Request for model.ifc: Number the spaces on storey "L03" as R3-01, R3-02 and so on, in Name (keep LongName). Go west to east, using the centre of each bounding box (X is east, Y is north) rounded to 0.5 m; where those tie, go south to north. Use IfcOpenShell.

First a look at what the model holds.

```python
import ifcopenshell
import ifcopenshell.util.element
import ifcopenshell.util.placement

model = ifcopenshell.open("model.ifc")
print(model.schema)
storey = next(s for s in model.by_type("IfcBuildingStorey") if s.Name == "L03")
spaces = [e for e in ifcopenshell.util.element.get_decomposition(storey) if e.is_a("IfcSpace")]
for e in sorted(spaces, key=lambda e: e.id()):
    origin = ifcopenshell.util.placement.get_local_placement(e.ObjectPlacement)[:3, 3]
    print(e.id(), e.Name, e.LongName, origin.round(2) + 0.0, sep=" | ")
```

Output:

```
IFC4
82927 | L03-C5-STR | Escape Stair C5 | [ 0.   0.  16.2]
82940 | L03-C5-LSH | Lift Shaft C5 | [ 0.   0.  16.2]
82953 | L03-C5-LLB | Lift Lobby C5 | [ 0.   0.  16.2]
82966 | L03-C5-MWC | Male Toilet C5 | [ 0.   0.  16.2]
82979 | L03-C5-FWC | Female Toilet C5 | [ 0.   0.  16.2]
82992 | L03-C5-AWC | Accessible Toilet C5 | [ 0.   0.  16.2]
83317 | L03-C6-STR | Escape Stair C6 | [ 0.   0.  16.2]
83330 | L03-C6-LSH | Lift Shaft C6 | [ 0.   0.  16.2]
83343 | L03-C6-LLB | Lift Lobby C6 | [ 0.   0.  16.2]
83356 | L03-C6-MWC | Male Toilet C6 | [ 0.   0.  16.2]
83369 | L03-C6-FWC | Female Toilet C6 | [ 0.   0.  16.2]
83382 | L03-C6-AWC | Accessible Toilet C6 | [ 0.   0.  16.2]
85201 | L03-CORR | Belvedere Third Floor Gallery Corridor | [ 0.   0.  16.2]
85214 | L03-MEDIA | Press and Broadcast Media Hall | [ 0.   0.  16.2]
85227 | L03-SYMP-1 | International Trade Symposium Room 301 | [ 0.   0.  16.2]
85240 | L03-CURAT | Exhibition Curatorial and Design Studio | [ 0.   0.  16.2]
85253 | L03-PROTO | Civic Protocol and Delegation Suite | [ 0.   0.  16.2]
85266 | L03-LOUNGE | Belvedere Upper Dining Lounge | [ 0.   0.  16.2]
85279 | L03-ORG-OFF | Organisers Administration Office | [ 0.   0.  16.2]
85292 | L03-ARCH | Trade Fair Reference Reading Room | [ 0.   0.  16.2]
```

```python
import ifcopenshell
import ifcopenshell.geom
import ifcopenshell.util.element
import ifcopenshell.util.shape

model = ifcopenshell.open("model.ifc")
settings = ifcopenshell.geom.settings()
settings.set("use-world-coords", True)


def centre(element):
    shape = ifcopenshell.geom.create_shape(settings, element)
    return ifcopenshell.util.shape.get_bbox_centroid(shape.geometry)


storey = next(s for s in model.by_type("IfcBuildingStorey") if s.Name == "L03")
spaces = [e for e in ifcopenshell.util.element.get_decomposition(storey) if e.is_a("IfcSpace")]

# Insertion points can sit at a corner or the storey origin, so sort by the geometry (in metres).
centres = {e: centre(e) for e in spaces}
spaces.sort(key=lambda e: (round(centres[e][0] / 0.5), centres[e][1]))

for i, e in enumerate(spaces, start=1):
    number = f"R3-{i:02d}"
    e.Name = number
    print(e.id(), number)

model.write("model_rev.ifc")
```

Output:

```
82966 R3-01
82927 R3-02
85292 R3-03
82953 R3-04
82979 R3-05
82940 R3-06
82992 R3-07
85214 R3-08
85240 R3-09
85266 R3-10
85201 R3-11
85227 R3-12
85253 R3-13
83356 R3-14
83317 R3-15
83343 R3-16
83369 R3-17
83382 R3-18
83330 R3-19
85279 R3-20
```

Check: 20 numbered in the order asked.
